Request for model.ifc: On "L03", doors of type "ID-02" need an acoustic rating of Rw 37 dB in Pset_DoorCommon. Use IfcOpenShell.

First a look at what the model holds.

```python
import ifcopenshell
import ifcopenshell.util.element

model = ifcopenshell.open("model.ifc")
print(model.schema)
storey = next(s for s in model.by_type("IfcBuildingStorey") if s.Name == "L03")
doors = [e for e in ifcopenshell.util.element.get_decomposition(storey) if e.is_a("IfcDoor")]
seen = {}
for e in doors:
    element_type = ifcopenshell.util.element.get_type(e)
    key = (element_type.Name if element_type != e and element_type else None, ifcopenshell.util.element.get_pset(e, "Pset_DoorCommon", "AcousticRating"))
    seen[key] = seen.get(key, 0) + 1
for (name, value), count in sorted(seen.items(), key=str):
    print(count, "x", name, "|", value)
```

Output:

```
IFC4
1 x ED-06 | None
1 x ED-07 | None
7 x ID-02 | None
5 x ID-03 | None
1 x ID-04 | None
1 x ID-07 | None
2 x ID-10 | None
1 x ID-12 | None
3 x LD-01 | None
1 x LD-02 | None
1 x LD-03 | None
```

```python
import ifcopenshell
import ifcopenshell.api.pset
import ifcopenshell.util.element

model = ifcopenshell.open("model.ifc")

storey = next(s for s in model.by_type("IfcBuildingStorey") if s.Name == "L03")
doors = [e for e in ifcopenshell.util.element.get_decomposition(storey) if e.is_a("IfcDoor")]

count = 0
for e in doors:
    element_type = ifcopenshell.util.element.get_type(e)
    if element_type in (None, e) or element_type.Name != "ID-02":
        continue
    # add_pset returns the element's existing set when there is one.
    pset = ifcopenshell.api.pset.add_pset(model, product=e, name="Pset_DoorCommon")
    ifcopenshell.api.pset.edit_pset(model, pset=pset, properties={"AcousticRating": "Rw 37 dB"})
    count += 1

print(count, "doors updated")

model.write("model_v2.ifc")
```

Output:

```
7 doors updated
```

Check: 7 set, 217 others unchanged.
